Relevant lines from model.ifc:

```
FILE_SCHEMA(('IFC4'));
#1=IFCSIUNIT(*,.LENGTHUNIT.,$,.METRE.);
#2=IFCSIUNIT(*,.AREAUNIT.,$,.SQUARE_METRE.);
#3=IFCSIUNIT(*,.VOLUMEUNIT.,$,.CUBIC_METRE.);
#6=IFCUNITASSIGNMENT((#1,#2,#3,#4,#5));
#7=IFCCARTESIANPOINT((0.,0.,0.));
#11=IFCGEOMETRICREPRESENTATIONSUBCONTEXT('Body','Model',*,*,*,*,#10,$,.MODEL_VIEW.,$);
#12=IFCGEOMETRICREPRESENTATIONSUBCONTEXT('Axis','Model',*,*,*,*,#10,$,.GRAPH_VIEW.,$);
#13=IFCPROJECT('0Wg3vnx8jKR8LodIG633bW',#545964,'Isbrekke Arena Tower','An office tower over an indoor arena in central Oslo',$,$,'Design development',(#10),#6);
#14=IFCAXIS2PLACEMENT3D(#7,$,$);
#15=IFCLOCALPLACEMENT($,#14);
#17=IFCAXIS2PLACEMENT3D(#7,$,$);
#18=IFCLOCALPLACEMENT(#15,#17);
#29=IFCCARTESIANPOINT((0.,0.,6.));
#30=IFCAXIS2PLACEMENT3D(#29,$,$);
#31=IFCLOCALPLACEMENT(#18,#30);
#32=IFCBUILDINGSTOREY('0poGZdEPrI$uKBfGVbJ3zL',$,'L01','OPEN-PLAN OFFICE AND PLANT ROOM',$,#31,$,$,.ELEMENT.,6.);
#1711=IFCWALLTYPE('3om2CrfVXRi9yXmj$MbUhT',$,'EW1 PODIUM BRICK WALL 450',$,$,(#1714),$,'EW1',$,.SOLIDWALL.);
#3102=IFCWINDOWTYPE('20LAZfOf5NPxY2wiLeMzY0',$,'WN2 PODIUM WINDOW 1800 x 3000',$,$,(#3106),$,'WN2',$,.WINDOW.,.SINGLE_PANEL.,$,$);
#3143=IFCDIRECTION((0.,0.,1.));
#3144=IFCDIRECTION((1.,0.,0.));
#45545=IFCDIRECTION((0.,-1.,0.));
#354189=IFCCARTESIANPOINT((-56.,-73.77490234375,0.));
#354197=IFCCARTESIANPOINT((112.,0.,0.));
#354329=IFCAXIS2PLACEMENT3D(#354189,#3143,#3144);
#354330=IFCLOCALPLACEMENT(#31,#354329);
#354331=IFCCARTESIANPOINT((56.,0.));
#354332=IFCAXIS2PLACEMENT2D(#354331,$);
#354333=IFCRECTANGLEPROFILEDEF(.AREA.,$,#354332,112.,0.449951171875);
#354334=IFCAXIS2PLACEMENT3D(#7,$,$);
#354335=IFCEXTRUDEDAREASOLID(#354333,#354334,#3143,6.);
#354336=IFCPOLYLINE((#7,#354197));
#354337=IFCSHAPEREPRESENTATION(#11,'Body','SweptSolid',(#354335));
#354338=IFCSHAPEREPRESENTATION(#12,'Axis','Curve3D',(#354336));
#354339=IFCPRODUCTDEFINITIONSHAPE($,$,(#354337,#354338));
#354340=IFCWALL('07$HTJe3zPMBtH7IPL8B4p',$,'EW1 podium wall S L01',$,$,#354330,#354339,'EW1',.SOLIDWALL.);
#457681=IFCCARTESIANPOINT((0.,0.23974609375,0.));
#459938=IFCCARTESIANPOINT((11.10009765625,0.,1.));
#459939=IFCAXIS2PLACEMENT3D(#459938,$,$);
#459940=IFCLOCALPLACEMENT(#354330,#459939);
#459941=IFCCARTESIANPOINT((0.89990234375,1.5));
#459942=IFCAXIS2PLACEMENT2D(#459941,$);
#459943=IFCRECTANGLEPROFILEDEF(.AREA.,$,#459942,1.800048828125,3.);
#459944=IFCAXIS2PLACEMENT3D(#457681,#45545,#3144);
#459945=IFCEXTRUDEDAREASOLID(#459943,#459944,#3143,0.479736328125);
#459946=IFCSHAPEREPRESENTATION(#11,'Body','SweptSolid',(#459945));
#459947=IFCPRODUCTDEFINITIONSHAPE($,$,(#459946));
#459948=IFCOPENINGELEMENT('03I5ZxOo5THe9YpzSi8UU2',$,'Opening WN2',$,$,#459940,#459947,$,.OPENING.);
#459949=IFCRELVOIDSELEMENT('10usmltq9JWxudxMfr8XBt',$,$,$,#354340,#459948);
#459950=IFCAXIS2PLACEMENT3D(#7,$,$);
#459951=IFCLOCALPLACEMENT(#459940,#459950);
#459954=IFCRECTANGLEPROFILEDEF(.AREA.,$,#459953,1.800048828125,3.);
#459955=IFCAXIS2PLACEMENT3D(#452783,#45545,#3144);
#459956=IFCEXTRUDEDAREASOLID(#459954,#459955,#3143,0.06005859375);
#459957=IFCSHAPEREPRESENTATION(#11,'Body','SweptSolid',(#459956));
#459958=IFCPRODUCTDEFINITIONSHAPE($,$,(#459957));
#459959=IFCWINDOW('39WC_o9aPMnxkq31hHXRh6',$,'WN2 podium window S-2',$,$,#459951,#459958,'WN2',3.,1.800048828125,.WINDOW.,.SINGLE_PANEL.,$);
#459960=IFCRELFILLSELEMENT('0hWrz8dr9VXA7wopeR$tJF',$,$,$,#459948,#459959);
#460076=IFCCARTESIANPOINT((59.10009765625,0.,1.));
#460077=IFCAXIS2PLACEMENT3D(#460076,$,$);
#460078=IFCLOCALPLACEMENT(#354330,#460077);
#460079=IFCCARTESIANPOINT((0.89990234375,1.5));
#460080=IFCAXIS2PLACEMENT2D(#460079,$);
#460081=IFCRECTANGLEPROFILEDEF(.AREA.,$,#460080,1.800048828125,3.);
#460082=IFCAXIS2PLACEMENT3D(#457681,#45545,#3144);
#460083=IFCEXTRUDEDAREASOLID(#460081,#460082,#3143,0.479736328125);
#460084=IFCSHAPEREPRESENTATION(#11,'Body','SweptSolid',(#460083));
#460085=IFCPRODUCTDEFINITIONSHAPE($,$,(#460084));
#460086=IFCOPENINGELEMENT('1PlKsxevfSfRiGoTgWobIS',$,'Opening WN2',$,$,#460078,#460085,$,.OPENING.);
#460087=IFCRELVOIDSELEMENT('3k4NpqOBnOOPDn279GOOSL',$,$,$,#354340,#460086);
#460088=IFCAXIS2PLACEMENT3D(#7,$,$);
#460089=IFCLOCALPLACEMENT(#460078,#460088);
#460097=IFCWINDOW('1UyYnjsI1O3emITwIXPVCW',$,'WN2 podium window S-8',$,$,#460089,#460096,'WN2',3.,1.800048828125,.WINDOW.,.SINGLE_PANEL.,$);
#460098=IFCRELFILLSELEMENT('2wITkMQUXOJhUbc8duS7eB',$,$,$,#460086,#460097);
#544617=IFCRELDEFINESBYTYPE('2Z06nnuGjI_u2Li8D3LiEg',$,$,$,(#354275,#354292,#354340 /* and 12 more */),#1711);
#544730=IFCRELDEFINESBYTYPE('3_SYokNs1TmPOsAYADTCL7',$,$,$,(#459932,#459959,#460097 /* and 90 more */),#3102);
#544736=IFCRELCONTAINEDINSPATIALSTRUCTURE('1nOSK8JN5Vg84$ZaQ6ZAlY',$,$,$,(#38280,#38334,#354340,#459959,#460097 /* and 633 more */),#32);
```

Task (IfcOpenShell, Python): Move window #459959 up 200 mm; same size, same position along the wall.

```python
import numpy as np
import ifcopenshell
import ifcopenshell.api.geometry
import ifcopenshell.util.placement
import ifcopenshell.util.unit

model = ifcopenshell.open("model.ifc")
unit_scale = ifcopenshell.util.unit.calculate_unit_scale(model)

window = model.by_id(459959)
opening = window.FillsVoids[0].RelatingOpeningElement
dz = 0.2

shift = np.array([0.0, 0.0, dz])
# The window is placed relative to its opening, so it follows when the opening moves.
matrix = ifcopenshell.util.placement.get_local_placement(opening.ObjectPlacement)
matrix[:3, 3] += shift
ifcopenshell.api.geometry.edit_object_placement(
    model, product=opening, matrix=matrix, is_si=False, should_transform_children=True
)

print(f"moved by {dz * unit_scale:+.3f} m")

model.write("model-out.ifc")
```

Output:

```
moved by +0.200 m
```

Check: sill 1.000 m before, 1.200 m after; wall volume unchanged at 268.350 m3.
